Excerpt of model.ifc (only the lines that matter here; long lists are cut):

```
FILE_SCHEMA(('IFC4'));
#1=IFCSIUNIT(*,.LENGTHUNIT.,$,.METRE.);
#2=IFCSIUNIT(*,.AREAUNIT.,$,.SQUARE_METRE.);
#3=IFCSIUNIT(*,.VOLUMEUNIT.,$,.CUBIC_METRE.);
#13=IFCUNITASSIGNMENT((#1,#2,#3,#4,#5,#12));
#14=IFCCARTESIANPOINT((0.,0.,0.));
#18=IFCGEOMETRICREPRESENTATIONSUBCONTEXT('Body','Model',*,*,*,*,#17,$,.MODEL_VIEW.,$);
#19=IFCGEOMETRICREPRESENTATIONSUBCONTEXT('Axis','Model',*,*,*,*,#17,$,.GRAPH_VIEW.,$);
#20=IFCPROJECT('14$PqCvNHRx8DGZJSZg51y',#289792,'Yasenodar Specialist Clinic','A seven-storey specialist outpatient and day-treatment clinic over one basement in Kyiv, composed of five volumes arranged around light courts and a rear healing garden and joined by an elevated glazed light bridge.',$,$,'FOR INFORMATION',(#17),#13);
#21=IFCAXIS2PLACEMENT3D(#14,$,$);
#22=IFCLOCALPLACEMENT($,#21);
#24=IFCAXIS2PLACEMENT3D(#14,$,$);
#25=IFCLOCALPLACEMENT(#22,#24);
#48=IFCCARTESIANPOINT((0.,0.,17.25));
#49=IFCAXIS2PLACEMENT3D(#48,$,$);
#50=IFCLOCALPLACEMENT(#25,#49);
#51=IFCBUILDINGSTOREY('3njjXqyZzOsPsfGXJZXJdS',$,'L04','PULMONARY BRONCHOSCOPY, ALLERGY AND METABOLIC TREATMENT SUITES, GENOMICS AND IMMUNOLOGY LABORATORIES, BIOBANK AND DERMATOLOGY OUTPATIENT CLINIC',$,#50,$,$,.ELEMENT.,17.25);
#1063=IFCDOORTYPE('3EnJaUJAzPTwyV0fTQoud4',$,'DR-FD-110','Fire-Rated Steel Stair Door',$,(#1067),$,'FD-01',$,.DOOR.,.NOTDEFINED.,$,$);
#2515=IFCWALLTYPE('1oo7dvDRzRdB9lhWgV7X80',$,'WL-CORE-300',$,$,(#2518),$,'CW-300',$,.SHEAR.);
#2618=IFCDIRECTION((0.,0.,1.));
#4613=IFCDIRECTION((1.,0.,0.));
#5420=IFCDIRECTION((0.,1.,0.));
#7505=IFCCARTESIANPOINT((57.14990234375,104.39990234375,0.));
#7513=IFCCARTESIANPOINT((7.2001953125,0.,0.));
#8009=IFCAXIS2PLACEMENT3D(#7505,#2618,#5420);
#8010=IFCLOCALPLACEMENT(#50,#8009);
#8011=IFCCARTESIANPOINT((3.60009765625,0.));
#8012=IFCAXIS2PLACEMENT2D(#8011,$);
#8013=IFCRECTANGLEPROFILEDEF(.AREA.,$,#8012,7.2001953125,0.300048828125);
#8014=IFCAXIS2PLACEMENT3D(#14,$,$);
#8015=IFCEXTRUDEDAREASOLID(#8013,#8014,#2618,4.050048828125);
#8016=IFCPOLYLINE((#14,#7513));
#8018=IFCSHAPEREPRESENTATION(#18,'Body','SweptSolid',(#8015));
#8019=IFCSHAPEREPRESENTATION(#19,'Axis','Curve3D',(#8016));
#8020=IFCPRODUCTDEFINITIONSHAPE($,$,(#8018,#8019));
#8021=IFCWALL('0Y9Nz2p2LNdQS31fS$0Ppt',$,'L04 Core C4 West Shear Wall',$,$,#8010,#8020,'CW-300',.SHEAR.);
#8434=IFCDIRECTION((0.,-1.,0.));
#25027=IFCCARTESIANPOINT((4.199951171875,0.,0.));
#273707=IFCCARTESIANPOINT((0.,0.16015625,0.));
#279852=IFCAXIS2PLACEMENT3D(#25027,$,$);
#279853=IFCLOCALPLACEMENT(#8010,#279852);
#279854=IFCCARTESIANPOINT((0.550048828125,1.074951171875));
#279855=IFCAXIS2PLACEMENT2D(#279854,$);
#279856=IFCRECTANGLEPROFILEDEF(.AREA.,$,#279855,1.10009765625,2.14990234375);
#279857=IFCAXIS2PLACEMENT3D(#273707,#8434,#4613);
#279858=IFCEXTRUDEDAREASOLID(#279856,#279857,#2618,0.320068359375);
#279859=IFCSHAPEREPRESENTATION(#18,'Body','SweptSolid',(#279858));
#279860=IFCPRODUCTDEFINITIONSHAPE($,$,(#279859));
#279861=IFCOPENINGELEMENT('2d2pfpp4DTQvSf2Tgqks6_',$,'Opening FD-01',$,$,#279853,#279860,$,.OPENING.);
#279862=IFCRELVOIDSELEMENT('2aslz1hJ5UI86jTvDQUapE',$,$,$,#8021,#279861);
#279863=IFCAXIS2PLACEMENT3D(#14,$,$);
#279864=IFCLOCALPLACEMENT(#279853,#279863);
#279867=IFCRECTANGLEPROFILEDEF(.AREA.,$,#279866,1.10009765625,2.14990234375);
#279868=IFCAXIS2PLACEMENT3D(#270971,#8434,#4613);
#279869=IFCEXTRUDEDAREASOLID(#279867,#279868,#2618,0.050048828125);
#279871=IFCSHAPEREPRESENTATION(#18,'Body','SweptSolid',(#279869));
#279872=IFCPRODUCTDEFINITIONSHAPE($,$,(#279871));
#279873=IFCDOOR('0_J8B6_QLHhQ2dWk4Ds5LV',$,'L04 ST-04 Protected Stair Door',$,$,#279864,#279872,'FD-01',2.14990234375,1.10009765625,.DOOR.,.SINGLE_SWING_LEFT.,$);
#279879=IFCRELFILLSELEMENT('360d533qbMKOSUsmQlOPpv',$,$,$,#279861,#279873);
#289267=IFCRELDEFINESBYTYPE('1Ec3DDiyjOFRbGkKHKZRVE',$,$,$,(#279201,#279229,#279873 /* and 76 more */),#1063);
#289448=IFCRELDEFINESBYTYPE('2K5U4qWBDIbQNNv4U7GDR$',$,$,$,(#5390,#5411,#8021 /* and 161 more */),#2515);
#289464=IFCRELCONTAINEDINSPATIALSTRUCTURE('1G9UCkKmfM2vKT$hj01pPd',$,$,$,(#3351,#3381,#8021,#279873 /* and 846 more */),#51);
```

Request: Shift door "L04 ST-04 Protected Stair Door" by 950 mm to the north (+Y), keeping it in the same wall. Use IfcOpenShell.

```python
import ifcopenshell
import ifcopenshell.api.geometry
import ifcopenshell.util.placement

model = ifcopenshell.open("model.ifc")

door = model.by_guid("0_J8B6_QLHhQ2dWk4Ds5LV")
opening = door.FillsVoids[0].RelatingOpeningElement
wall = opening.VoidsElements[0].RelatingBuildingElement

wall_matrix = ifcopenshell.util.placement.get_local_placement(wall.ObjectPlacement)
shift = wall_matrix[:3, 0] * 0.95
before = ifcopenshell.util.placement.get_local_placement(door.ObjectPlacement)[:3, 3].copy()

# The door is placed relative to its opening, so it follows when the opening moves.
matrix = ifcopenshell.util.placement.get_local_placement(opening.ObjectPlacement)
matrix[:3, 3] += shift
ifcopenshell.api.geometry.edit_object_placement(
    model, product=opening, matrix=matrix, is_si=False, should_transform_children=True
)

after = ifcopenshell.util.placement.get_local_placement(door.ObjectPlacement)[:3, 3]
print("door moved by", (after - before).round(3) + 0.0)

model.write("model_rev.ifc")
```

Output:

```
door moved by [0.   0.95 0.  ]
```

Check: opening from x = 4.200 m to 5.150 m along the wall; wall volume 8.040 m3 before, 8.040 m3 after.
